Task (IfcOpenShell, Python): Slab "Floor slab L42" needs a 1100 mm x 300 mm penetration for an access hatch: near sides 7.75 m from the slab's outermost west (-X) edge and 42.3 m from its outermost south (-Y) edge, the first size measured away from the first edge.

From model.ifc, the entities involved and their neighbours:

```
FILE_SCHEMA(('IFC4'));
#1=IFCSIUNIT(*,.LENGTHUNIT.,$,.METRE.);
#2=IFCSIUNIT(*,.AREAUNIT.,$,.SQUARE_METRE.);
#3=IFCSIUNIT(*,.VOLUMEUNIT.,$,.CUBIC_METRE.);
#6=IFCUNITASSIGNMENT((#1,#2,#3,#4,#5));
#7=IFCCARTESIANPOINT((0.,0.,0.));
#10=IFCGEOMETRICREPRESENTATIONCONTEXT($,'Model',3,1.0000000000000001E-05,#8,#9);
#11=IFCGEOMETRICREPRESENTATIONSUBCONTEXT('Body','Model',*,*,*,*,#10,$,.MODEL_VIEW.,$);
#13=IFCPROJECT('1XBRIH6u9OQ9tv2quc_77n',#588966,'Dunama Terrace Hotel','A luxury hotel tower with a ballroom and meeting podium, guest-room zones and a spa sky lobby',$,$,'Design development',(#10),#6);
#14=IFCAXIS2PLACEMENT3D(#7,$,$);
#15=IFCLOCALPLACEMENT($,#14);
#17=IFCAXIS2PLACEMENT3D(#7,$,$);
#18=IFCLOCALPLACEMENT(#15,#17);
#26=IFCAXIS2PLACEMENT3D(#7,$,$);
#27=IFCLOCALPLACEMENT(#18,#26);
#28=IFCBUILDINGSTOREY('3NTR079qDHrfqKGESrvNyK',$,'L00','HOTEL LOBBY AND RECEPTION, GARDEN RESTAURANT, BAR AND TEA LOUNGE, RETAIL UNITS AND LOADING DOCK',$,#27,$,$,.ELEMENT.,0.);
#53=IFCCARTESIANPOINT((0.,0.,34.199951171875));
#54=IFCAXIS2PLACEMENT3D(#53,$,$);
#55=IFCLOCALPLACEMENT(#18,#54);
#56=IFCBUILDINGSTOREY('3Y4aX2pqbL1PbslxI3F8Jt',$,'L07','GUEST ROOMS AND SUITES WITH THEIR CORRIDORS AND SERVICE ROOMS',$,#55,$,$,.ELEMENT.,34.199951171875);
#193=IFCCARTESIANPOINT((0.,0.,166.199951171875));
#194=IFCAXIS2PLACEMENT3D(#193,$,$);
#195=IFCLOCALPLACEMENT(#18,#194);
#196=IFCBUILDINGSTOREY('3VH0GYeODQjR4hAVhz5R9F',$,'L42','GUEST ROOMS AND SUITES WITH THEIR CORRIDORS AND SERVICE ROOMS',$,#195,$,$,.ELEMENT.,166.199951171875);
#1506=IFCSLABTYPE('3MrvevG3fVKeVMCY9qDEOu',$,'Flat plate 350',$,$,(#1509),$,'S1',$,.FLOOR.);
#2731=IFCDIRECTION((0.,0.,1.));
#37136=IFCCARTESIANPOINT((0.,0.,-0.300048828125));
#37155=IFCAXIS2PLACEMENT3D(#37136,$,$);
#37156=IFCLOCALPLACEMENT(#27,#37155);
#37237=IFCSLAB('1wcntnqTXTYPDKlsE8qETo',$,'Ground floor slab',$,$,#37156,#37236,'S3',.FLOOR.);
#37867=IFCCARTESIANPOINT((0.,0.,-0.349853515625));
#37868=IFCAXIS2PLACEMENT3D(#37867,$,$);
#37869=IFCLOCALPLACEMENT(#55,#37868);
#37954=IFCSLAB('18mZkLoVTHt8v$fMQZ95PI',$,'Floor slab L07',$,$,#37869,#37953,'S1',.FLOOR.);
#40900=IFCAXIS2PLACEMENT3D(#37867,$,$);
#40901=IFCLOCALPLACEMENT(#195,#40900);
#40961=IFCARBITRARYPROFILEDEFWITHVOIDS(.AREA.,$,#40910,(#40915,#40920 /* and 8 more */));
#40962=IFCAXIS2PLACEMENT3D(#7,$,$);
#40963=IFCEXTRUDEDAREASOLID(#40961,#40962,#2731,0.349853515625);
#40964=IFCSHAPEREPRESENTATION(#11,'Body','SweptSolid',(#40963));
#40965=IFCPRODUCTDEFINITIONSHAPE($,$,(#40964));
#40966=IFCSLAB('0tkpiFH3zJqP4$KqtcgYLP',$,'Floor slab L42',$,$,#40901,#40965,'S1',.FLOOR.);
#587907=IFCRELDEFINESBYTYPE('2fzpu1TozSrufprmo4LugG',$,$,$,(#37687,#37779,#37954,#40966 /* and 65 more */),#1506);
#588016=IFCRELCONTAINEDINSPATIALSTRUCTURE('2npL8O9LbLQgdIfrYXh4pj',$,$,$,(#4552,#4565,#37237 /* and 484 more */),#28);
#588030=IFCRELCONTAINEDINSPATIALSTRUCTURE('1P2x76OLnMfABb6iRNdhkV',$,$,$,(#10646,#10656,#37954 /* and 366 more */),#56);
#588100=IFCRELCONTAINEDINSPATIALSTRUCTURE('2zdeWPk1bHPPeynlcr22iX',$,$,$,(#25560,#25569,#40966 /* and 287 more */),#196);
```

```python
import numpy as np
import ifcopenshell
import ifcopenshell.api.feature
import ifcopenshell.api.geometry
import ifcopenshell.api.root
import ifcopenshell.geom
import ifcopenshell.util.placement
import ifcopenshell.util.representation
import ifcopenshell.util.shape
import ifcopenshell.util.unit

model = ifcopenshell.open("model.ifc")
unit_scale = ifcopenshell.util.unit.calculate_unit_scale(model)
settings = ifcopenshell.geom.settings()


def volume(element):
    """Net volume in cubic metres, openings subtracted."""
    shape = ifcopenshell.geom.create_shape(settings, element)
    return ifcopenshell.util.shape.get_volume(shape.geometry)


slab = model.by_guid("0tkpiFH3zJqP4$KqtcgYLP")
before = volume(slab)

# Extent in the slab's own axes, in metres. The edges named are its -X and -Y sides.
slab_shape = ifcopenshell.geom.create_shape(settings, slab)
vertices = ifcopenshell.util.shape.get_vertices(slab_shape.geometry)
x_min, y_min, bottom = vertices.min(axis=0)
top = vertices[:, 2].max()

opening = ifcopenshell.api.root.create_entity(model, ifc_class="IfcOpeningElement", name="Access hatch opening", predefined_type="OPENING")
context = ifcopenshell.util.representation.get_context(model, "Model", "Body", "MODEL_VIEW")
width, depth = 1.1, 0.3
outline = [(0.0, 0.0), (width, 0.0), (width, depth), (0.0, depth), (0.0, 0.0)]
# Overshoot both faces by 50 mm so the cut is clean.
shape = ifcopenshell.api.geometry.add_slab_representation(
    model, context=context, depth=top - bottom + 0.1, polyline=outline
)
ifcopenshell.api.geometry.assign_representation(model, product=opening, representation=shape)

matrix = ifcopenshell.util.placement.get_local_placement(slab.ObjectPlacement)
matrix[:, 3] = matrix @ np.append(np.array([x_min + 7.75, y_min + 42.3, bottom - 0.05]) / unit_scale, 1.0)
ifcopenshell.api.geometry.edit_object_placement(model, product=opening, matrix=matrix, is_si=False)
ifcopenshell.api.feature.add_feature(model, feature=opening, element=slab)

after = volume(slab)

print(f"slab volume {before:.3f} -> {after:.3f} m3")

model.write("model_rev.ifc")
```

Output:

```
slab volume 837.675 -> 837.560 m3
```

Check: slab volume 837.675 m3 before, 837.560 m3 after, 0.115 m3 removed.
